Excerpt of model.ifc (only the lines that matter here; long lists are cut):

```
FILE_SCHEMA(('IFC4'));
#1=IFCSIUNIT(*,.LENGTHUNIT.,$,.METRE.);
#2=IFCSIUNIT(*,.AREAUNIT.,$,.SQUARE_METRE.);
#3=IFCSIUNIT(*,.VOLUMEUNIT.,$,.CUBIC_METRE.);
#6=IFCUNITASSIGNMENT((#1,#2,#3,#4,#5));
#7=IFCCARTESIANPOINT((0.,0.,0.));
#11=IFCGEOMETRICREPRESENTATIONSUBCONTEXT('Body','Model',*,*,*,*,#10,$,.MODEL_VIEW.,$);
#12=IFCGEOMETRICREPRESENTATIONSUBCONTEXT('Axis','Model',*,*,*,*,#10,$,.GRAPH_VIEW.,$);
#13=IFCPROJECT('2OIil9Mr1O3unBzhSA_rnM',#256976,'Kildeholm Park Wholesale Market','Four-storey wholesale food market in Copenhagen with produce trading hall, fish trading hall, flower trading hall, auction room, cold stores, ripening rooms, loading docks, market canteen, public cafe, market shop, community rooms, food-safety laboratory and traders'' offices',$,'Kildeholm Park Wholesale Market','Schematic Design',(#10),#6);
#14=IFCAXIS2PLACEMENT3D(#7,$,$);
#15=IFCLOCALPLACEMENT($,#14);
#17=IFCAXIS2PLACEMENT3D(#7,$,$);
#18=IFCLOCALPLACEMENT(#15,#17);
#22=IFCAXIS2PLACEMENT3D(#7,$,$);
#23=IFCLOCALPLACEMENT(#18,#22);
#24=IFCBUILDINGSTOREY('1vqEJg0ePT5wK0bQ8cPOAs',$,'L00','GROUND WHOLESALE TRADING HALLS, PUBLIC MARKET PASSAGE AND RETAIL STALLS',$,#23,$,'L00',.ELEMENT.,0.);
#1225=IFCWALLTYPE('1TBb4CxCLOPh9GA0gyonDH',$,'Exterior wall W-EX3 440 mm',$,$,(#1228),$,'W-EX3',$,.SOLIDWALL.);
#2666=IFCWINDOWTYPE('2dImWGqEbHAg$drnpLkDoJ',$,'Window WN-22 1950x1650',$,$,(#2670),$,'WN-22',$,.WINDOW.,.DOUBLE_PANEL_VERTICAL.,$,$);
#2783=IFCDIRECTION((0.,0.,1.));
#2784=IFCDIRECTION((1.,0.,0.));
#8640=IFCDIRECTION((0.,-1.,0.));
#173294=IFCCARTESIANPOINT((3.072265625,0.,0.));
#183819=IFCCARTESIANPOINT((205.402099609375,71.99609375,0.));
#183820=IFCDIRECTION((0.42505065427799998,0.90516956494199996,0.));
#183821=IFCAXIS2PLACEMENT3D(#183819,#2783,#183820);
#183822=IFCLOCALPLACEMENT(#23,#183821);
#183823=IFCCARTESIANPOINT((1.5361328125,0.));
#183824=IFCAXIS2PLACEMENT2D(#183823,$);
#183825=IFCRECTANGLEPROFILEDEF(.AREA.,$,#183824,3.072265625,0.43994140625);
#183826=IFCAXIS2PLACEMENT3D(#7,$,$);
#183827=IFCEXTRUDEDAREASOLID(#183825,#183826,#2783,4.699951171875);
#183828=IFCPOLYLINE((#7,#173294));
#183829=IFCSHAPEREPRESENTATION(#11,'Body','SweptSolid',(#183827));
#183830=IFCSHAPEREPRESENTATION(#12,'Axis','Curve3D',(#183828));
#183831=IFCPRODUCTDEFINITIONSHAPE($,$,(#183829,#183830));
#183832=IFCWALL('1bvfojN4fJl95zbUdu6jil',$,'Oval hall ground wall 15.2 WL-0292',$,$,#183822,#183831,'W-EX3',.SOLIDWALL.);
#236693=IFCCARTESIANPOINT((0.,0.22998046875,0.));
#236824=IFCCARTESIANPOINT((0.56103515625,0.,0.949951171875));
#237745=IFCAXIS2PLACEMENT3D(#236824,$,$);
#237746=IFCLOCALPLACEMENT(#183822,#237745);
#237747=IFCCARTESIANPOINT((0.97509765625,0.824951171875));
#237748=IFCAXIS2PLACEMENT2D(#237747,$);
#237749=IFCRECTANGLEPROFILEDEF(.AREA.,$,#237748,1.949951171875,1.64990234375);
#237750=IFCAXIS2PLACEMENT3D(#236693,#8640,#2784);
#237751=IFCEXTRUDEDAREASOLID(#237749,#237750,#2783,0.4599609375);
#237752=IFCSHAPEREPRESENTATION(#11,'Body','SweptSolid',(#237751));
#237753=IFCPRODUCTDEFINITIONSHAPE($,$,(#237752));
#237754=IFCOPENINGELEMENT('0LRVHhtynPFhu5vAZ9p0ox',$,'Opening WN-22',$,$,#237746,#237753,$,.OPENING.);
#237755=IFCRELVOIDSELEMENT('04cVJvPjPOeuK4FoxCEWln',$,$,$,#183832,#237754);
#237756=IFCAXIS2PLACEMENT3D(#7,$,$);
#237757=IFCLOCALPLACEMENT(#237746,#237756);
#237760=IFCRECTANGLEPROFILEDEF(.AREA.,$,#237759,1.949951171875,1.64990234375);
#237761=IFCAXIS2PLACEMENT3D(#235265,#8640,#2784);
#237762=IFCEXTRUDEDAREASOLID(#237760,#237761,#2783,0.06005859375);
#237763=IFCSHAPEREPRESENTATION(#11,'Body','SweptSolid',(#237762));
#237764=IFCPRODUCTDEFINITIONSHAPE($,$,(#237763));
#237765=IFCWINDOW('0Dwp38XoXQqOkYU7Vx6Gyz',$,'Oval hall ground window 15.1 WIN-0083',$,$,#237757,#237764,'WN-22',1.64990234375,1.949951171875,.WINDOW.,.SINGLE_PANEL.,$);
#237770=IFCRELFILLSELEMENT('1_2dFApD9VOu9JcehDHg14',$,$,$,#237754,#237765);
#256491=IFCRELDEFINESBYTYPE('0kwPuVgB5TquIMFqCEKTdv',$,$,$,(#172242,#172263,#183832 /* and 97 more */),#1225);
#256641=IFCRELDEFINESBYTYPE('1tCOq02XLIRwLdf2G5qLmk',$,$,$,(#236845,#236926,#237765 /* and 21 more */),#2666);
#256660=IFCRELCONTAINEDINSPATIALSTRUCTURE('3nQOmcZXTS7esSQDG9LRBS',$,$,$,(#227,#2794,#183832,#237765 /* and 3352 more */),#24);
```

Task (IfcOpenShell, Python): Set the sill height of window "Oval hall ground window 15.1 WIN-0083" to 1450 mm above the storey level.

```python
import numpy as np
import ifcopenshell
import ifcopenshell.api.geometry
import ifcopenshell.geom
import ifcopenshell.util.element
import ifcopenshell.util.placement
import ifcopenshell.util.shape
import ifcopenshell.util.unit

model = ifcopenshell.open("model.ifc")
unit_scale = ifcopenshell.util.unit.calculate_unit_scale(model)

window = model.by_guid("0Dwp38XoXQqOkYU7Vx6Gyz")
opening = window.FillsVoids[0].RelatingOpeningElement
storey = ifcopenshell.util.element.get_container(window, ifc_class="IfcBuildingStorey")
level = ifcopenshell.util.placement.get_local_placement(storey.ObjectPlacement)[2, 3]

# The opening's origin need not be at the sill, so measure its lowest point.
shape = ifcopenshell.geom.create_shape(ifcopenshell.geom.settings(), opening)
bottom = ifcopenshell.util.shape.get_shape_bottom_elevation(shape, shape.geometry) / unit_scale
dz = level + 1.45 - bottom

shift = np.array([0.0, 0.0, dz])
# The window is placed relative to its opening, so it follows when the opening moves.
matrix = ifcopenshell.util.placement.get_local_placement(opening.ObjectPlacement)
matrix[:3, 3] += shift
ifcopenshell.api.geometry.edit_object_placement(
    model, product=opening, matrix=matrix, is_si=False, should_transform_children=True
)

print(f"moved by {dz * unit_scale:+.3f} m")

model.write("model_edited.ifc")
```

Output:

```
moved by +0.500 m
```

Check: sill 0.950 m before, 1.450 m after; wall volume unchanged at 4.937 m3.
